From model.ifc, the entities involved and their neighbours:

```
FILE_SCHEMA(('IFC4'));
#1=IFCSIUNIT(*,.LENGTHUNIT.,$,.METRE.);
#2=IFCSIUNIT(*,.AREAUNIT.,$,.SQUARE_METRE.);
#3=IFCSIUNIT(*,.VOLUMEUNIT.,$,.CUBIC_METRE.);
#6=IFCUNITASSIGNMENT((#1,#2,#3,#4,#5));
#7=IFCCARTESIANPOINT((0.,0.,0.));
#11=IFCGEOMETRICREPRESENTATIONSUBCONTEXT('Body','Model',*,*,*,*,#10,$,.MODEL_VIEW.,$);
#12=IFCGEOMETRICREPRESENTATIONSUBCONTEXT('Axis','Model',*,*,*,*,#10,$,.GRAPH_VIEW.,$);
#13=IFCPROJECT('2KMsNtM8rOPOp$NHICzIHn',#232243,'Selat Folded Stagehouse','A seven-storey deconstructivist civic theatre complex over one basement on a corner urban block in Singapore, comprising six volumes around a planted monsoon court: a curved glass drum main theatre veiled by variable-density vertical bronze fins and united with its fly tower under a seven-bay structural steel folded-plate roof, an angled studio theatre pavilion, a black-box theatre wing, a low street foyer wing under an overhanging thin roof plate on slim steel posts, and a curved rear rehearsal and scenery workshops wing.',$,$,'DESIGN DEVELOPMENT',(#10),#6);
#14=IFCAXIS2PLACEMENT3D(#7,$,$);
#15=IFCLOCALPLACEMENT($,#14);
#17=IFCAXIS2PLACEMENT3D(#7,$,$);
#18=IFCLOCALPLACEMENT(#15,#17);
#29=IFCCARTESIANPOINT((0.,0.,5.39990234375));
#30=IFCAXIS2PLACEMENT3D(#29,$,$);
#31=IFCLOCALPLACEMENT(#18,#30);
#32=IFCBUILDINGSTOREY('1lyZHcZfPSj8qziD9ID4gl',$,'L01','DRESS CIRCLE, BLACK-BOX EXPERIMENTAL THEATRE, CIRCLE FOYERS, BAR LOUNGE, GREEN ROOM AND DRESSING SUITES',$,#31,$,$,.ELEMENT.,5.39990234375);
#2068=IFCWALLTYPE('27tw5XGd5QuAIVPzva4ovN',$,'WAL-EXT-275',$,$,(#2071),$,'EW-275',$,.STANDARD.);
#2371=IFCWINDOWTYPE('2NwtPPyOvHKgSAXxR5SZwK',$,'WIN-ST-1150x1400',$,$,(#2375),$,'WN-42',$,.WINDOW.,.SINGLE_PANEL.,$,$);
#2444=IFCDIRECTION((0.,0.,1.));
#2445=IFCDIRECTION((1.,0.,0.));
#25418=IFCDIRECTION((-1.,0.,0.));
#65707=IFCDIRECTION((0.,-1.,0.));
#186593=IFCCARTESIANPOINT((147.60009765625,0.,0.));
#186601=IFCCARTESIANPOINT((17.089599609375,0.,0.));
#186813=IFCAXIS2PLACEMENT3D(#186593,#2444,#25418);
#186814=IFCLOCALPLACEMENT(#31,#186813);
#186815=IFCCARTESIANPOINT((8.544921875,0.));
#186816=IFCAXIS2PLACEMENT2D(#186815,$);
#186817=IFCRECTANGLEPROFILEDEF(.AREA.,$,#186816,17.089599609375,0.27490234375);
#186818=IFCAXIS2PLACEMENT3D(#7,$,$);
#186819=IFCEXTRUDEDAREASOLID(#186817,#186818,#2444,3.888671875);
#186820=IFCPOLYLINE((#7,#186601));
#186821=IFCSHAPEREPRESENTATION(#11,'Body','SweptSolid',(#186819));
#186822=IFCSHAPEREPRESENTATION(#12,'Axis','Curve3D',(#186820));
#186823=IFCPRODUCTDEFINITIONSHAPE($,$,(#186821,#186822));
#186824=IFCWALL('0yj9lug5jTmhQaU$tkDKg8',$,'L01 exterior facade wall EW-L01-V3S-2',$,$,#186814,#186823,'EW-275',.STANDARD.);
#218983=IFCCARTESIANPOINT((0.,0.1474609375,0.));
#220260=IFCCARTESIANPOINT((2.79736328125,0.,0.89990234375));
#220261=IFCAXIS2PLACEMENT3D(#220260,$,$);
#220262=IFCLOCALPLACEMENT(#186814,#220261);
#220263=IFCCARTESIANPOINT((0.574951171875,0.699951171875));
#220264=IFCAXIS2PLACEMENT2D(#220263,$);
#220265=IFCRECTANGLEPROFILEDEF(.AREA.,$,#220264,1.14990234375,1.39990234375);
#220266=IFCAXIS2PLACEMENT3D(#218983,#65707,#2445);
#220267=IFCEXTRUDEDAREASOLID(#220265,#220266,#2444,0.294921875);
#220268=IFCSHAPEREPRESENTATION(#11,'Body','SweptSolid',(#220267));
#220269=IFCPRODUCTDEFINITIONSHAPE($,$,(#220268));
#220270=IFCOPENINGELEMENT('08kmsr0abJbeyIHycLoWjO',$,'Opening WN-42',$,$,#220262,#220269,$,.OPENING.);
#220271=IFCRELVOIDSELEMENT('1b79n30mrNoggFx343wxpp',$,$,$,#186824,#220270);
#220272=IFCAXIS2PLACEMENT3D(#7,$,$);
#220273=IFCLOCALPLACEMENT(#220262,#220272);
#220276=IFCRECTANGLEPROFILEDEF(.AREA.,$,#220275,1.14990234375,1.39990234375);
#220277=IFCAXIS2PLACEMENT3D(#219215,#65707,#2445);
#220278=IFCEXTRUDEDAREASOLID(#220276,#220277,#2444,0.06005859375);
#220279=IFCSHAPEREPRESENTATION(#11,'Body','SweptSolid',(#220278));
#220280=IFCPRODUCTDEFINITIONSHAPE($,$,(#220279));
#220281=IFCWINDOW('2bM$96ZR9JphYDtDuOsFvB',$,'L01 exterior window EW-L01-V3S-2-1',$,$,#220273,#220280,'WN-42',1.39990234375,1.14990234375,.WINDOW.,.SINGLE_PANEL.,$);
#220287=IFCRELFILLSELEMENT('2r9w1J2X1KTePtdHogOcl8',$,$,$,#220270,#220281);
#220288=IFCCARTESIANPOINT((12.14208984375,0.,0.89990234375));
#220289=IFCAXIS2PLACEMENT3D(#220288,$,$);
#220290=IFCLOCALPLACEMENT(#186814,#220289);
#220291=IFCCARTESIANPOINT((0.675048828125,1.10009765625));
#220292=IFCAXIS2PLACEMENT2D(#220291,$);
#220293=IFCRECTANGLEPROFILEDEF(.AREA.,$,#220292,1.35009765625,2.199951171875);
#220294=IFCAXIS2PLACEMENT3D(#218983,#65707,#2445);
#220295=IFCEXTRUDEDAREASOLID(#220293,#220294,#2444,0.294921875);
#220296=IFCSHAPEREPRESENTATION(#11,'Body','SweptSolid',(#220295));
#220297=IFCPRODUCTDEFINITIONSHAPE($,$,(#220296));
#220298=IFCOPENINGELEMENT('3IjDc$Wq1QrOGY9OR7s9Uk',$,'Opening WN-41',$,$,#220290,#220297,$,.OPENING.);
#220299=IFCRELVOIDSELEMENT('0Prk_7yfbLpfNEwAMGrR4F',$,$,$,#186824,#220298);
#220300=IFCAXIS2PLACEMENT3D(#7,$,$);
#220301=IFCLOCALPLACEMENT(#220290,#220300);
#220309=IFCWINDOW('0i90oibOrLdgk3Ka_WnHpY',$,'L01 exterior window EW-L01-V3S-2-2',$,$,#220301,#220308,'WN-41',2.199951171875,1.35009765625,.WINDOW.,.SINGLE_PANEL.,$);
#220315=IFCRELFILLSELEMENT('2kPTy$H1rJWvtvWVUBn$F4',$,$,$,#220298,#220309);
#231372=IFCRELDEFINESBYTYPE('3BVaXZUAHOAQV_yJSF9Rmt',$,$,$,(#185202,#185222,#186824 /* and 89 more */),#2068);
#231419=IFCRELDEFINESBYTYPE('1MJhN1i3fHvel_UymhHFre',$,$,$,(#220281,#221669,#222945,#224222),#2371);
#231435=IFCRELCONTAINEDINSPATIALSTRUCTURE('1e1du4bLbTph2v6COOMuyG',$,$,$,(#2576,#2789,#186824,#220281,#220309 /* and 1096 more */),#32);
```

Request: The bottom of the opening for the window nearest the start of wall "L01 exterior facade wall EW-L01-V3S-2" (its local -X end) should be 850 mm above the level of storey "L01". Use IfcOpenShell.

```python
import numpy as np
import ifcopenshell
import ifcopenshell.api.geometry
import ifcopenshell.geom
import ifcopenshell.util.element
import ifcopenshell.util.placement
import ifcopenshell.util.shape
import ifcopenshell.util.unit

model = ifcopenshell.open("model.ifc")
unit_scale = ifcopenshell.util.unit.calculate_unit_scale(model)

window = model.by_guid("2bM$96ZR9JphYDtDuOsFvB")
opening = window.FillsVoids[0].RelatingOpeningElement
storey = ifcopenshell.util.element.get_container(window, ifc_class="IfcBuildingStorey")
level = ifcopenshell.util.placement.get_local_placement(storey.ObjectPlacement)[2, 3]

# The opening's origin need not be at the sill, so measure its lowest point.
shape = ifcopenshell.geom.create_shape(ifcopenshell.geom.settings(), opening)
bottom = ifcopenshell.util.shape.get_shape_bottom_elevation(shape, shape.geometry) / unit_scale
dz = level + 0.85 - bottom

shift = np.array([0.0, 0.0, dz])
# The window is placed relative to its opening, so it follows when the opening moves.
matrix = ifcopenshell.util.placement.get_local_placement(opening.ObjectPlacement)
matrix[:3, 3] += shift
ifcopenshell.api.geometry.edit_object_placement(
    model, product=opening, matrix=matrix, is_si=False, should_transform_children=True
)

print(f"moved by {dz * unit_scale:+.3f} m")

model.write("model_v2.ifc")
```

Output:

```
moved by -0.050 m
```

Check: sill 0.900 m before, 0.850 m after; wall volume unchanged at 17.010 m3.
